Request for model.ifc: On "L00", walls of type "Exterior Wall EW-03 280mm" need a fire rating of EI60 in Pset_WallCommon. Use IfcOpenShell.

First a look at what the model holds.

```python
import ifcopenshell
import ifcopenshell.util.element

model = ifcopenshell.open("model.ifc")
print(model.schema)
storey = next(s for s in model.by_type("IfcBuildingStorey") if s.Name == "L00")
walls = [e for e in ifcopenshell.util.element.get_decomposition(storey) if e.is_a("IfcWall")]
seen = {}
for e in walls:
    element_type = ifcopenshell.util.element.get_type(e)
    key = (element_type.Name if element_type != e and element_type else None, ifcopenshell.util.element.get_pset(e, "Pset_WallCommon", "FireRating"))
    seen[key] = seen.get(key, 0) + 1
for (name, value), count in sorted(seen.items(), key=str):
    print(count, "x", name, "|", value)
```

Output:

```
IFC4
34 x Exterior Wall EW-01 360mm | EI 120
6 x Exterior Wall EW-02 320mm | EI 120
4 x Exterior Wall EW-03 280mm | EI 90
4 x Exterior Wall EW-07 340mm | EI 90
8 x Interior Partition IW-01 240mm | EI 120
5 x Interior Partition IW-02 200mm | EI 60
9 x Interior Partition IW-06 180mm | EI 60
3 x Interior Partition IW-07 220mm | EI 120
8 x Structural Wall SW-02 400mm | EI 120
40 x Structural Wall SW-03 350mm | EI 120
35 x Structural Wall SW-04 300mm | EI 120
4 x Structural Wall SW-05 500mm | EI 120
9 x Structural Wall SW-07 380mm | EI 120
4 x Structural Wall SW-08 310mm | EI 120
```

```python
import ifcopenshell
import ifcopenshell.api.pset
import ifcopenshell.util.element

model = ifcopenshell.open("model.ifc")

storey = next(s for s in model.by_type("IfcBuildingStorey") if s.Name == "L00")
walls = [e for e in ifcopenshell.util.element.get_decomposition(storey) if e.is_a("IfcWall")]

count = 0
for e in walls:
    element_type = ifcopenshell.util.element.get_type(e)
    if element_type in (None, e) or element_type.Name != "Exterior Wall EW-03 280mm":
        continue
    # add_pset returns the element's existing set when there is one.
    pset = ifcopenshell.api.pset.add_pset(model, product=e, name="Pset_WallCommon")
    ifcopenshell.api.pset.edit_pset(model, pset=pset, properties={"FireRating": "EI60"})
    count += 1

print(count, "walls updated")

model.write("model_rev.ifc")
```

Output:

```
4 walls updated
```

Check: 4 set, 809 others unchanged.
